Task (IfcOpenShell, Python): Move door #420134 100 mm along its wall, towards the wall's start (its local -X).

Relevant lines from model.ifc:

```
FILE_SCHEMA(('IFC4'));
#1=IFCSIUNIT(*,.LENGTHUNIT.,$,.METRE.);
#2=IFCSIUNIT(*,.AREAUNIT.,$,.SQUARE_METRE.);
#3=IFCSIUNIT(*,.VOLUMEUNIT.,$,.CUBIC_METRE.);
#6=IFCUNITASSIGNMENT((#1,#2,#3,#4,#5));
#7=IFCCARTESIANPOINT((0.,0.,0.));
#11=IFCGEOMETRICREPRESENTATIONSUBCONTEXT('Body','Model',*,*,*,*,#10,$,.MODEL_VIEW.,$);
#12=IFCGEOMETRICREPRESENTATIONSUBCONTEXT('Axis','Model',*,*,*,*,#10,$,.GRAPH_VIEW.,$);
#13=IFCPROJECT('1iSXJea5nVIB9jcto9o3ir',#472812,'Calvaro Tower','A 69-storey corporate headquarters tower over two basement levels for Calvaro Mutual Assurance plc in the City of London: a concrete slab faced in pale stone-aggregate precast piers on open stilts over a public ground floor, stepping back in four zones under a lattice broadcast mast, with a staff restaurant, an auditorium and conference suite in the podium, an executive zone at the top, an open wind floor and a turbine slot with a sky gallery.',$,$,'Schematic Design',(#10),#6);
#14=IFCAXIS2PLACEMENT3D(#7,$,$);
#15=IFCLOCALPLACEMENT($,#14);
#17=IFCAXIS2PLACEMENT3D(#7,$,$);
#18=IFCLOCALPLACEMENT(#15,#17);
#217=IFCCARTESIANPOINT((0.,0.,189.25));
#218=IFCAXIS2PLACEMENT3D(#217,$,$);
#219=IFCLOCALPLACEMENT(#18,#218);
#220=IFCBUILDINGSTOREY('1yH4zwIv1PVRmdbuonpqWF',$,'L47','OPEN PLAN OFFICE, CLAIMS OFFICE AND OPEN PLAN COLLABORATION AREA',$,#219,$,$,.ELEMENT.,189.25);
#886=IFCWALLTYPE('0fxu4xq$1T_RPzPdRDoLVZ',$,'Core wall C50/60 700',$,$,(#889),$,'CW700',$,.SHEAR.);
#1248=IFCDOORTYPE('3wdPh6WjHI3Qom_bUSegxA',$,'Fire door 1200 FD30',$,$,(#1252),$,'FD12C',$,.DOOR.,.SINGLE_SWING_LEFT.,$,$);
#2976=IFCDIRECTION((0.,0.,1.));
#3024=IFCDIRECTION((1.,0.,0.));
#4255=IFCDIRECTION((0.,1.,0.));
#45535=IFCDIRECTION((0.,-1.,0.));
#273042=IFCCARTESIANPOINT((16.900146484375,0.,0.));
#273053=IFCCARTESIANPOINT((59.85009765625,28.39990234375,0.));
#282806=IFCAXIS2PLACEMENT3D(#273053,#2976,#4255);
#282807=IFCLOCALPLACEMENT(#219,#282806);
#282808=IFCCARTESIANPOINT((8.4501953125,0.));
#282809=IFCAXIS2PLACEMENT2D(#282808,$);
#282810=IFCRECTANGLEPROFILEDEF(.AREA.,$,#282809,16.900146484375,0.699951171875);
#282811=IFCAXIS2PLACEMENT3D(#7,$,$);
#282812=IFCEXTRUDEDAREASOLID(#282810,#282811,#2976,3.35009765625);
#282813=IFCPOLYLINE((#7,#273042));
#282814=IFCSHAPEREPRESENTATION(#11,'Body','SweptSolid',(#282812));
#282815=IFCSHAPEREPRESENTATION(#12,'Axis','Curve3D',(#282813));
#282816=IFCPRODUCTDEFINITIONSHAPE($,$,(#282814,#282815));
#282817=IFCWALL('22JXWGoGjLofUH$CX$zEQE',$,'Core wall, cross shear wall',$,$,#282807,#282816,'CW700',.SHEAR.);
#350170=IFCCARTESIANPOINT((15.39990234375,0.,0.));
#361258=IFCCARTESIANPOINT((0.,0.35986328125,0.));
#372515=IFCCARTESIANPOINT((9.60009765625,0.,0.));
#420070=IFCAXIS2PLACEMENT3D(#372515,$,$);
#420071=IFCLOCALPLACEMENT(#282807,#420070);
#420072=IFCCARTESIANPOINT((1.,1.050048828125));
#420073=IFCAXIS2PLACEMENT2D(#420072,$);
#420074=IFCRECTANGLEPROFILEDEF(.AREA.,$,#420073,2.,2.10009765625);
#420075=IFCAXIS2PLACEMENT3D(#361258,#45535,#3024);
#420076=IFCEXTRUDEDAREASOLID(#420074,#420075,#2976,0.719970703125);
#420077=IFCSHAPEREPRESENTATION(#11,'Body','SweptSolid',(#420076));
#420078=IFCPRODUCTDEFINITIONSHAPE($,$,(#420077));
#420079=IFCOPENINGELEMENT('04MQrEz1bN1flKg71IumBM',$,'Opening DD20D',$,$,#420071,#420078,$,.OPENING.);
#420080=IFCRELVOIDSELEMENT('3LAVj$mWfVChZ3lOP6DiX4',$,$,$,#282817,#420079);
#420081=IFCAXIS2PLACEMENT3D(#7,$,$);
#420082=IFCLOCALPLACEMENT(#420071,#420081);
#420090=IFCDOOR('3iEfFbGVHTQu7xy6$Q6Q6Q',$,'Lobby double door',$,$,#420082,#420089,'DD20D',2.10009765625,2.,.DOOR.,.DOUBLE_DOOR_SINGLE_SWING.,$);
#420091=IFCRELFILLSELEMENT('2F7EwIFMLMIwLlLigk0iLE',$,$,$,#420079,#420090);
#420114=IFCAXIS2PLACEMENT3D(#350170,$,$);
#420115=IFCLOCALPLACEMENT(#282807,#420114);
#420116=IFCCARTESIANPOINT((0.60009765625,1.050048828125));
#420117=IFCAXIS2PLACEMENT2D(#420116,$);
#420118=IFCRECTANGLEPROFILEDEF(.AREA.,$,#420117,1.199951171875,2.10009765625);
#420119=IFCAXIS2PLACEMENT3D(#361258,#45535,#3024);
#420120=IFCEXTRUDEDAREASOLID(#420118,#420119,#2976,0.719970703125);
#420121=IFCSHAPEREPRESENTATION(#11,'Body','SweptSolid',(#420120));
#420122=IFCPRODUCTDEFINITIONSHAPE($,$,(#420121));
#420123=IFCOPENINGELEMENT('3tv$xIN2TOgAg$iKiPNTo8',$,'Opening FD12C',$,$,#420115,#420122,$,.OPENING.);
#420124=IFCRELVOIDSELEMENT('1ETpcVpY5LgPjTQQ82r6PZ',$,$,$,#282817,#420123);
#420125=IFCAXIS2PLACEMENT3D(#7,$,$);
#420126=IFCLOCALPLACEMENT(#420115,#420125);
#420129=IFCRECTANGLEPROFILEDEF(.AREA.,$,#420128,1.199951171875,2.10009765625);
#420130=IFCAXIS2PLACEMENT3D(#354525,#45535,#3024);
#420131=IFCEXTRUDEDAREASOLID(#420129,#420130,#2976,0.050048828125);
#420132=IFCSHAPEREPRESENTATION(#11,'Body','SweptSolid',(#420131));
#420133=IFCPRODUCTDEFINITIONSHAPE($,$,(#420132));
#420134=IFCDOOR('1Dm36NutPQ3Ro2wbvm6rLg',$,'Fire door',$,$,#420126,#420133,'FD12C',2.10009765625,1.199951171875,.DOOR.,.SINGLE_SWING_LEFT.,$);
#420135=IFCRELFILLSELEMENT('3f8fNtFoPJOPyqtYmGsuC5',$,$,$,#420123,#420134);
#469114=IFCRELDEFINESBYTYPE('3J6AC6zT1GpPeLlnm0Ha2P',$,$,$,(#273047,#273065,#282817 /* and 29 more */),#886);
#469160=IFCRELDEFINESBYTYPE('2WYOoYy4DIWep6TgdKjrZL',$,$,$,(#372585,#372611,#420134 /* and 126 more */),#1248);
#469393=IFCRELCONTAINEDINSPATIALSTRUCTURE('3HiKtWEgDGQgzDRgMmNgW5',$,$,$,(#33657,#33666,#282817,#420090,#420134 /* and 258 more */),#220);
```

```python
import ifcopenshell
import ifcopenshell.api.geometry
import ifcopenshell.util.placement
import ifcopenshell.util.unit

model = ifcopenshell.open("model.ifc")
unit_scale = ifcopenshell.util.unit.calculate_unit_scale(model)

door = model.by_guid("1Dm36NutPQ3Ro2wbvm6rLg")
opening = door.FillsVoids[0].RelatingOpeningElement
wall = opening.VoidsElements[0].RelatingBuildingElement

wall_matrix = ifcopenshell.util.placement.get_local_placement(wall.ObjectPlacement)
shift = wall_matrix[:3, 0] * -0.1 / unit_scale
before = ifcopenshell.util.placement.get_local_placement(door.ObjectPlacement)[:3, 3].copy()

# The door is placed relative to its opening, so it follows when the opening moves.
matrix = ifcopenshell.util.placement.get_local_placement(opening.ObjectPlacement)
matrix[:3, 3] += shift
ifcopenshell.api.geometry.edit_object_placement(
    model, product=opening, matrix=matrix, is_si=False, should_transform_children=True
)

after = ifcopenshell.util.placement.get_local_placement(door.ObjectPlacement)[:3, 3]
print("door moved by", (after - before).round(3) + 0.0)

model.write("model_updated.ifc")
```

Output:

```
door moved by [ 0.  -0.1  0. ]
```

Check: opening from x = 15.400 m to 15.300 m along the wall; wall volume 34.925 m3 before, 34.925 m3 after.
